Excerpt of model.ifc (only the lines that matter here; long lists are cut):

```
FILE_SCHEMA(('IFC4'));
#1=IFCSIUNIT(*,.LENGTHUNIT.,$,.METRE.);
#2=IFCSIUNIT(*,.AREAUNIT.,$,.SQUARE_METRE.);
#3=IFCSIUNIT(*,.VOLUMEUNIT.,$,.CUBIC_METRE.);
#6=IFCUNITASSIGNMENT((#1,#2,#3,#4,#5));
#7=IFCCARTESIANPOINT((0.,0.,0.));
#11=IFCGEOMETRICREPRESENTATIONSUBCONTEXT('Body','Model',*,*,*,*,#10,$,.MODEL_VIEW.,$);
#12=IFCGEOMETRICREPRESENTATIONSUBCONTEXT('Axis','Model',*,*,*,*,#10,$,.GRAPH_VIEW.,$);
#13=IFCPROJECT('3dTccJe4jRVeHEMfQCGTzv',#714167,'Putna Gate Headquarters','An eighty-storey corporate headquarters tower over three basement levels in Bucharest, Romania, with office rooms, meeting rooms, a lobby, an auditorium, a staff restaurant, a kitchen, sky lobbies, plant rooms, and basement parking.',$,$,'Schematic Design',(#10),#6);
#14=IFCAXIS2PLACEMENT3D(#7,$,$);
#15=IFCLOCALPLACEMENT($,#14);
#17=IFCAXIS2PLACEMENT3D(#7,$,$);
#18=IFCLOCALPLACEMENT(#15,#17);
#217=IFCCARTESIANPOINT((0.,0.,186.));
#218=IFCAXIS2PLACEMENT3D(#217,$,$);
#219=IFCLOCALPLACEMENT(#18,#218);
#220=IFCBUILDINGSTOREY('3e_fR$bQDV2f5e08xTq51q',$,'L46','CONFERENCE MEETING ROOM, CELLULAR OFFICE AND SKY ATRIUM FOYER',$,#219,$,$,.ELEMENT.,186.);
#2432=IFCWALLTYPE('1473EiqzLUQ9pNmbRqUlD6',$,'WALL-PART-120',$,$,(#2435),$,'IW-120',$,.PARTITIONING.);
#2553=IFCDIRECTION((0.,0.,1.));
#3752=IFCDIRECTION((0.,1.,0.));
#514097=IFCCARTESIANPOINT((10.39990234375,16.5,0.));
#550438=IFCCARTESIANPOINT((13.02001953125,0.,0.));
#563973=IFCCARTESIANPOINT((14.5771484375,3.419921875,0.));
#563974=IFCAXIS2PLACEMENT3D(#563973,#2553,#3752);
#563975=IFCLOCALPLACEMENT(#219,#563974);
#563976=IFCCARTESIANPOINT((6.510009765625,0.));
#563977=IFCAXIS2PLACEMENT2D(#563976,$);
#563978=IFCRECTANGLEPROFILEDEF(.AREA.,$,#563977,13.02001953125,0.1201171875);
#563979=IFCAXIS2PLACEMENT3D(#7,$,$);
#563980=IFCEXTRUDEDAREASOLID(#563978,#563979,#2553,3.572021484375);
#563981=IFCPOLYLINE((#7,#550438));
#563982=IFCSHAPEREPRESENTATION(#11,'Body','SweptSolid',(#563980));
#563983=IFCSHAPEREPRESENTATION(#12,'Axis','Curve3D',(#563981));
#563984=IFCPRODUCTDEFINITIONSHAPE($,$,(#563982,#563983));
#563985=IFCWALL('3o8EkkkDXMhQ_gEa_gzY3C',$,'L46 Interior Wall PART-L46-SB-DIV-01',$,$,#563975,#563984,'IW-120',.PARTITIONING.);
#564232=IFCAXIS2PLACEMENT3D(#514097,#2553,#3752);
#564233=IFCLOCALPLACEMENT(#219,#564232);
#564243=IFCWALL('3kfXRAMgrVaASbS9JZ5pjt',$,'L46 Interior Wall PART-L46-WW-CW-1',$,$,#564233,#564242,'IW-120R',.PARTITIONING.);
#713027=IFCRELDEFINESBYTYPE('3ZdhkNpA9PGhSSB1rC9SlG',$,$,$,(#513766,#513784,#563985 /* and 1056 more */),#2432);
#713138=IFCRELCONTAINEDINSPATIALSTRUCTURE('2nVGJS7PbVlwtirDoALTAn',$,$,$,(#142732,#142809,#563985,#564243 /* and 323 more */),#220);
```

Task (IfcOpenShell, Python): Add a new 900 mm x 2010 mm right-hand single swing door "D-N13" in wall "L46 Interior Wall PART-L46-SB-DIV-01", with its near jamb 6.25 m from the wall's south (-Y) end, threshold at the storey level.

```python
import numpy as np
import ifcopenshell
import ifcopenshell.api.feature
import ifcopenshell.api.geometry
import ifcopenshell.api.root
import ifcopenshell.api.spatial
import ifcopenshell.geom
import ifcopenshell.util.element
import ifcopenshell.util.placement
import ifcopenshell.util.representation
import ifcopenshell.util.shape
import ifcopenshell.util.unit

model = ifcopenshell.open("model.ifc")
unit_scale = ifcopenshell.util.unit.calculate_unit_scale(model)
settings = ifcopenshell.geom.settings()


def volume(element):
    """Net volume in cubic metres, openings subtracted."""
    shape = ifcopenshell.geom.create_shape(settings, element)
    return ifcopenshell.util.shape.get_volume(shape.geometry)


wall = model.by_guid("3o8EkkkDXMhQ_gEa_gzY3C")
storey = ifcopenshell.util.element.get_container(wall, ifc_class="IfcBuildingStorey")
context = ifcopenshell.util.representation.get_context(model, "Model", "Body", "MODEL_VIEW")
before = volume(wall)

width, height, from_end, sill = 0.9, 2.01, 6.25, 0.0  # metres

# The wall runs along its own X axis, and the end named is its -X end.
wall_shape = ifcopenshell.geom.create_shape(settings, wall)
x, y, z = ifcopenshell.util.shape.get_vertices(wall_shape.geometry).T
start = x.min() + from_end
face, thickness = float(y.min()), float(y.max() - y.min())
wall_matrix = ifcopenshell.util.placement.get_local_placement(wall.ObjectPlacement)
level = ifcopenshell.util.placement.get_local_placement(storey.ObjectPlacement)[2, 3]


def in_wall(x, y):
    """Placement at x, y metres in the wall's axes, at sill height."""
    matrix = wall_matrix.copy()
    matrix[:, 3] = wall_matrix @ np.array([x / unit_scale, y / unit_scale, 0.0, 1.0])
    matrix[2, 3] = level + sill / unit_scale
    return matrix


# Opening: a box that overshoots both wall faces by 50 mm.
opening = ifcopenshell.api.root.create_entity(model, ifc_class="IfcOpeningElement", predefined_type="OPENING")
box = ifcopenshell.api.geometry.add_wall_representation(
    model, context=context, length=width, height=height, thickness=thickness + 0.1
)
ifcopenshell.api.geometry.assign_representation(model, product=opening, representation=box)
ifcopenshell.api.geometry.edit_object_placement(model, product=opening, matrix=in_wall(start, face - 0.05), is_si=False)
ifcopenshell.api.feature.add_feature(model, feature=opening, element=wall)

door = ifcopenshell.api.root.create_entity(model, ifc_class="IfcDoor", name="D-N13", predefined_type="DOOR")
door.OverallWidth, door.OverallHeight = width / unit_scale, height / unit_scale
door.OperationType = "SINGLE_SWING_RIGHT"
body = ifcopenshell.api.geometry.add_door_representation(
    model,
    context=context,
    overall_width=door.OverallWidth,
    overall_height=door.OverallHeight,
    operation_type="SINGLE_SWING_RIGHT",
    lining_properties={"LiningDepth": thickness / unit_scale, "ThresholdDepth": thickness / unit_scale},
)
ifcopenshell.api.geometry.assign_representation(model, product=door, representation=body)
ifcopenshell.api.spatial.assign_container(model, products=[door], relating_structure=storey)
ifcopenshell.api.feature.add_filling(model, opening=opening, element=door)

# The lining spans the wall, so the door starts at the wall face.
ifcopenshell.api.geometry.edit_object_placement(model, product=door, matrix=in_wall(start, face), is_si=False)

after = volume(wall)

print(f"wall volume {before:.3f} -> {after:.3f} m3")

model.write("model_rev.ifc")
```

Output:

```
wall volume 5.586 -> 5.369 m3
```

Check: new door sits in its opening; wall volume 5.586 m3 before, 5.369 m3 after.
